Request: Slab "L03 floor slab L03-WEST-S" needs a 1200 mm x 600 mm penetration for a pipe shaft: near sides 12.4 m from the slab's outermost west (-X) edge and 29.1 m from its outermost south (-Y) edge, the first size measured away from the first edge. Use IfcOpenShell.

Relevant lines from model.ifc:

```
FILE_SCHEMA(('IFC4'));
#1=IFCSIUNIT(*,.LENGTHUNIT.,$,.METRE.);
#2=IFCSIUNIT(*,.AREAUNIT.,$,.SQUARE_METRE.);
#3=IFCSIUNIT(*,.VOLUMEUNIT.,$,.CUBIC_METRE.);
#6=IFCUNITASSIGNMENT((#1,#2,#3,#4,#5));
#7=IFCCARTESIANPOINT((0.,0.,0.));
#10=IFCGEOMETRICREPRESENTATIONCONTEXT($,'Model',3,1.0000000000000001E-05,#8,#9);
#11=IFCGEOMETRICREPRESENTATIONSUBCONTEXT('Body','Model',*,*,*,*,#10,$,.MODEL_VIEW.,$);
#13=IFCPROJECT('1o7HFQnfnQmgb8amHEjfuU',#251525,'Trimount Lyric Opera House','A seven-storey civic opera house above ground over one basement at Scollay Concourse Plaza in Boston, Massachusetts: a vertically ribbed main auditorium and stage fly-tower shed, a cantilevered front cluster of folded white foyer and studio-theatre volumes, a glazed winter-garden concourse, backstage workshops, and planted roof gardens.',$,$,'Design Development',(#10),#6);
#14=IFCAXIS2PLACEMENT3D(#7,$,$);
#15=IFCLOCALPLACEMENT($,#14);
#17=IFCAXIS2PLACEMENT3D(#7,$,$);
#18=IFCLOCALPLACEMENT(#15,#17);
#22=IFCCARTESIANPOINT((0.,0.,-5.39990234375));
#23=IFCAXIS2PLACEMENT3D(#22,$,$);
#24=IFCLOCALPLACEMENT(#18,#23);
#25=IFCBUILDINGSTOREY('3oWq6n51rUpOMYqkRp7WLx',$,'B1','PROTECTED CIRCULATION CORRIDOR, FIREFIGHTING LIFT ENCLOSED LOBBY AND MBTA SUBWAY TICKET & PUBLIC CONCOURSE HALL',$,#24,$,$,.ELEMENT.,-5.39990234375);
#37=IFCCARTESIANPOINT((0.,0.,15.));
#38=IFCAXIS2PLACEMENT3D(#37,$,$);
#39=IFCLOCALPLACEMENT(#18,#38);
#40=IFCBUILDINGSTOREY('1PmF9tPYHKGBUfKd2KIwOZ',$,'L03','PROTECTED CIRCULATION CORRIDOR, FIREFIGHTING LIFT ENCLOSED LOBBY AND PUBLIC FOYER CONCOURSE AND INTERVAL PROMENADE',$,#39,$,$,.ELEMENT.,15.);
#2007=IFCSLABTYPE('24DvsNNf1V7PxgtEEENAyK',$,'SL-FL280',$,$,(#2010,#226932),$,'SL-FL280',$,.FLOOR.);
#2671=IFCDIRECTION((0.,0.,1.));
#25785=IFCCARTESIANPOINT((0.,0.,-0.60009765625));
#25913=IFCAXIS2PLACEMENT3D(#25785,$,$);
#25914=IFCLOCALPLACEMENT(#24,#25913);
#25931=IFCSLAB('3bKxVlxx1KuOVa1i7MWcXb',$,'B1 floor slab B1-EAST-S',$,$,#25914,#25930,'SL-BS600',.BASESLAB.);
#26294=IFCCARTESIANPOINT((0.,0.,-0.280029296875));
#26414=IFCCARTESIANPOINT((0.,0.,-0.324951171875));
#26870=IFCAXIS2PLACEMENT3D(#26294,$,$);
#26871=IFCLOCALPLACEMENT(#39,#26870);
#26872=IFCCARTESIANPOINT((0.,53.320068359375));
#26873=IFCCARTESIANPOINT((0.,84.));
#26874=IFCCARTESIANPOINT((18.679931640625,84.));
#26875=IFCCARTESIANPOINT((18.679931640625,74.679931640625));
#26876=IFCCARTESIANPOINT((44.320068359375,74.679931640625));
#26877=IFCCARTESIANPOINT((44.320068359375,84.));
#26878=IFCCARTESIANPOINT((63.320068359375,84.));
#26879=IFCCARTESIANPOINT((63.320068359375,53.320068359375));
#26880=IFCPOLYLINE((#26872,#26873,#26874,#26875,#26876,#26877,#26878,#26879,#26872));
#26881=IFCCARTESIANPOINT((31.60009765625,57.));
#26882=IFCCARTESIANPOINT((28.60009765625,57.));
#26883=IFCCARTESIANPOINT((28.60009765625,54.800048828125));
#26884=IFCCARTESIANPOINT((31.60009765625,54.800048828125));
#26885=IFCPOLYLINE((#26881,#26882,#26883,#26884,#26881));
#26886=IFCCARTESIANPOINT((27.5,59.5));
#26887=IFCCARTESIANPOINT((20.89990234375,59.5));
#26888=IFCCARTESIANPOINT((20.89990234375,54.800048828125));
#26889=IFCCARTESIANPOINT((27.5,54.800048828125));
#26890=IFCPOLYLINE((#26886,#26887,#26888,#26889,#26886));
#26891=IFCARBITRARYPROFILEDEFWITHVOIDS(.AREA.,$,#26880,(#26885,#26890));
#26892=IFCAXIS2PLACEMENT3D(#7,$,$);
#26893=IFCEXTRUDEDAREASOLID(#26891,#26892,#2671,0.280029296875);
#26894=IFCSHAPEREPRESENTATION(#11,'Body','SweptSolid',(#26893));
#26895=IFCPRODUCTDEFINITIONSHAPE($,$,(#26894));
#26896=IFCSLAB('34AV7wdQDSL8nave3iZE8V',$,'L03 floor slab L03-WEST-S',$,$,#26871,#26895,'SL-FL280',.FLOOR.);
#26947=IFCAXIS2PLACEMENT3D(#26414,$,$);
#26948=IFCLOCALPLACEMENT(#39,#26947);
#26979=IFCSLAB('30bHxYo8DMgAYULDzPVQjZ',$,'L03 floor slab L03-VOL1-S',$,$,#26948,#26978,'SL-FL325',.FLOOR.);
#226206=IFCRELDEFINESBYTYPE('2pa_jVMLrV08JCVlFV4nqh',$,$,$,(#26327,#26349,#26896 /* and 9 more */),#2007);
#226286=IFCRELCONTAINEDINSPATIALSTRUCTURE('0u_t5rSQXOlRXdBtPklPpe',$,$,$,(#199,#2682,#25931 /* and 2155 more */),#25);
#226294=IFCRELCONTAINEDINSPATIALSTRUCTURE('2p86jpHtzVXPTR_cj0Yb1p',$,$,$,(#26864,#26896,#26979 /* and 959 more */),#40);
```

```python
import numpy as np
import ifcopenshell
import ifcopenshell.api.feature
import ifcopenshell.api.geometry
import ifcopenshell.api.root
import ifcopenshell.geom
import ifcopenshell.util.placement
import ifcopenshell.util.representation
import ifcopenshell.util.shape
import ifcopenshell.util.unit

model = ifcopenshell.open("model.ifc")
unit_scale = ifcopenshell.util.unit.calculate_unit_scale(model)
settings = ifcopenshell.geom.settings()


def volume(element):
    """Net volume in cubic metres, openings subtracted."""
    shape = ifcopenshell.geom.create_shape(settings, element)
    return ifcopenshell.util.shape.get_volume(shape.geometry)


slab = model.by_guid("34AV7wdQDSL8nave3iZE8V")
before = volume(slab)

# Extent in the slab's own axes, in metres. The edges named are its -X and -Y sides.
slab_shape = ifcopenshell.geom.create_shape(settings, slab)
vertices = ifcopenshell.util.shape.get_vertices(slab_shape.geometry)
x_min, y_min, bottom = vertices.min(axis=0)
top = vertices[:, 2].max()

opening = ifcopenshell.api.root.create_entity(model, ifc_class="IfcOpeningElement", name="Pipe shaft opening", predefined_type="OPENING")
context = ifcopenshell.util.representation.get_context(model, "Model", "Body", "MODEL_VIEW")
width, depth = 1.2, 0.6
outline = [(0.0, 0.0), (width, 0.0), (width, depth), (0.0, depth), (0.0, 0.0)]
# Overshoot both faces by 50 mm so the cut is clean.
shape = ifcopenshell.api.geometry.add_slab_representation(
    model, context=context, depth=top - bottom + 0.1, polyline=outline
)
ifcopenshell.api.geometry.assign_representation(model, product=opening, representation=shape)

matrix = ifcopenshell.util.placement.get_local_placement(slab.ObjectPlacement)
matrix[:, 3] = matrix @ np.append(np.array([x_min + 12.4, y_min + 29.1, bottom - 0.05]) / unit_scale, 1.0)
ifcopenshell.api.geometry.edit_object_placement(model, product=opening, matrix=matrix, is_si=False)
ifcopenshell.api.feature.add_feature(model, feature=opening, element=slab)

after = volume(slab)

print(f"slab volume {before:.3f} -> {after:.3f} m3")

model.write("model_updated.ifc")
```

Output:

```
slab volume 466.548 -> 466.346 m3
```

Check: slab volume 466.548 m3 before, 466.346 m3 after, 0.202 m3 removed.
